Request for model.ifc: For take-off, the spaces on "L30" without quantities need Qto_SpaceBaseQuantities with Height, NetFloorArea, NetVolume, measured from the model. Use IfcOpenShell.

First a look at what the model holds.

```python
import ifcopenshell
import ifcopenshell.util.element
import ifcopenshell.util.unit

model = ifcopenshell.open("model.ifc")
print(model.schema)
for unit_type in ("LENGTHUNIT", "AREAUNIT", "VOLUMEUNIT"):
    print(unit_type, ifcopenshell.util.unit.calculate_unit_scale(model, unit_type))
storey = next(s for s in model.by_type("IfcBuildingStorey") if s.Name == "L30")
spaces = [e for e in ifcopenshell.util.element.get_decomposition(storey) if e.is_a("IfcSpace")]
for e in sorted(spaces, key=lambda e: e.id()):
    print(e.id(), e.is_a(), e.Name, list(ifcopenshell.util.element.get_psets(e, qtos_only=True)), sep=" | ")
```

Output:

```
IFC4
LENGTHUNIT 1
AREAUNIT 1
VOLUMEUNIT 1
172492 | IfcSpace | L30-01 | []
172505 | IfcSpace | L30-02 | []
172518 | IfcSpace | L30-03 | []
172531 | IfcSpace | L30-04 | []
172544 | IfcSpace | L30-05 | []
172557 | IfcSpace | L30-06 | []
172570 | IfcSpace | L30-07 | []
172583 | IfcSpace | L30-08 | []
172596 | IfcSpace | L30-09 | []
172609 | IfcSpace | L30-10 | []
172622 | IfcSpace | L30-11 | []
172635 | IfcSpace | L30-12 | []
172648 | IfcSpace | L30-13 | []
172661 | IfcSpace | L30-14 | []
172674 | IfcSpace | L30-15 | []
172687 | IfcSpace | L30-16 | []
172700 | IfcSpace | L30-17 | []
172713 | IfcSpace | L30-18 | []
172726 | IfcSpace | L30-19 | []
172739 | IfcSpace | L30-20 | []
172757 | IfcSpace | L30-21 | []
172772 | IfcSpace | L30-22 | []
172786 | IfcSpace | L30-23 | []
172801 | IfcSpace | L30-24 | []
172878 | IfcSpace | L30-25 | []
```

```python
import ifcopenshell
import ifcopenshell.api.pset
import ifcopenshell.geom
import ifcopenshell.util.element
import ifcopenshell.util.shape
import ifcopenshell.util.unit

model = ifcopenshell.open("model.ifc")
unit_scale = ifcopenshell.util.unit.calculate_unit_scale(model)
area_scale = ifcopenshell.util.unit.calculate_unit_scale(model, "AREAUNIT")
volume_scale = ifcopenshell.util.unit.calculate_unit_scale(model, "VOLUMEUNIT")
settings = ifcopenshell.geom.settings()

storey = next(s for s in model.by_type("IfcBuildingStorey") if s.Name == "L30")
spaces = [e for e in ifcopenshell.util.element.get_decomposition(storey) if e.is_a("IfcSpace")]

for e in sorted(spaces, key=lambda e: e.id()):
    if ifcopenshell.util.element.get_psets(e, qtos_only=True, should_inherit=False):
        continue
    # Geometry comes back in metres, in the element's own axes.
    shape = ifcopenshell.geom.create_shape(settings, e)
    values = {
        "Height": ifcopenshell.util.shape.get_z(shape.geometry) / unit_scale,
        "NetFloorArea": ifcopenshell.util.shape.get_footprint_area(shape.geometry) / area_scale,
        "NetVolume": ifcopenshell.util.shape.get_volume(shape.geometry) / volume_scale,
    }
    qto = ifcopenshell.api.pset.add_qto(model, product=e, name="Qto_SpaceBaseQuantities")
    ifcopenshell.api.pset.edit_qto(model, qto=qto, properties=values)
    print(e.id(), {k: round(v, 3) for k, v in values.items()})

model.write("model_updated.ifc")
```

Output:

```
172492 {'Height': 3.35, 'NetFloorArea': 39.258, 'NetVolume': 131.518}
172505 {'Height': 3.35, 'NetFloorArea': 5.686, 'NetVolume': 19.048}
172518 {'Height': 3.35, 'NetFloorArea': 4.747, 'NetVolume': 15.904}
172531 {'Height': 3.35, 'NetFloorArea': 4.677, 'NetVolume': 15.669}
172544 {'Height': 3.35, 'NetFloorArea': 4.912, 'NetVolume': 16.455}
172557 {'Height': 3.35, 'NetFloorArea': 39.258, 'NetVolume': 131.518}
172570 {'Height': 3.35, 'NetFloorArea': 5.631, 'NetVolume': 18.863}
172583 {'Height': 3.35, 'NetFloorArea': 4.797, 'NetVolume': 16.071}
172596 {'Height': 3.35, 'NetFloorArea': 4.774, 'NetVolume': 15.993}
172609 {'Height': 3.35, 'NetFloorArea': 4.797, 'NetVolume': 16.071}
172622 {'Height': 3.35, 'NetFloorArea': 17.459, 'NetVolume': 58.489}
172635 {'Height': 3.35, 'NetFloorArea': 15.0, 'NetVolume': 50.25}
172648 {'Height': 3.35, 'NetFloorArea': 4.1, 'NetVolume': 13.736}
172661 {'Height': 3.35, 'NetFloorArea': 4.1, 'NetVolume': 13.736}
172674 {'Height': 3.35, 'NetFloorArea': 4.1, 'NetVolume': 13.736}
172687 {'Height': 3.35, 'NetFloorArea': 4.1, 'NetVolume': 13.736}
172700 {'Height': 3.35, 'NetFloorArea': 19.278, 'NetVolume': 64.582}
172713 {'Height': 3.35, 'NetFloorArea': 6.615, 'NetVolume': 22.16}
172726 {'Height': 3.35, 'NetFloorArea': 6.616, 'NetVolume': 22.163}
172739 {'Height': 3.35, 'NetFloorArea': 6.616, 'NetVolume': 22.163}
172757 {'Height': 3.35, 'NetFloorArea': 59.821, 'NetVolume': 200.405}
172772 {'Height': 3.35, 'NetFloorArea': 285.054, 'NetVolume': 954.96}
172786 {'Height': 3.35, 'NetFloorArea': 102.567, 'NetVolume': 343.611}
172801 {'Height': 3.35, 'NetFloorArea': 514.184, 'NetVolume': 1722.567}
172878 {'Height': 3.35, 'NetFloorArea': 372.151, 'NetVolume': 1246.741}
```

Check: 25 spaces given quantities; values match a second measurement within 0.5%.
